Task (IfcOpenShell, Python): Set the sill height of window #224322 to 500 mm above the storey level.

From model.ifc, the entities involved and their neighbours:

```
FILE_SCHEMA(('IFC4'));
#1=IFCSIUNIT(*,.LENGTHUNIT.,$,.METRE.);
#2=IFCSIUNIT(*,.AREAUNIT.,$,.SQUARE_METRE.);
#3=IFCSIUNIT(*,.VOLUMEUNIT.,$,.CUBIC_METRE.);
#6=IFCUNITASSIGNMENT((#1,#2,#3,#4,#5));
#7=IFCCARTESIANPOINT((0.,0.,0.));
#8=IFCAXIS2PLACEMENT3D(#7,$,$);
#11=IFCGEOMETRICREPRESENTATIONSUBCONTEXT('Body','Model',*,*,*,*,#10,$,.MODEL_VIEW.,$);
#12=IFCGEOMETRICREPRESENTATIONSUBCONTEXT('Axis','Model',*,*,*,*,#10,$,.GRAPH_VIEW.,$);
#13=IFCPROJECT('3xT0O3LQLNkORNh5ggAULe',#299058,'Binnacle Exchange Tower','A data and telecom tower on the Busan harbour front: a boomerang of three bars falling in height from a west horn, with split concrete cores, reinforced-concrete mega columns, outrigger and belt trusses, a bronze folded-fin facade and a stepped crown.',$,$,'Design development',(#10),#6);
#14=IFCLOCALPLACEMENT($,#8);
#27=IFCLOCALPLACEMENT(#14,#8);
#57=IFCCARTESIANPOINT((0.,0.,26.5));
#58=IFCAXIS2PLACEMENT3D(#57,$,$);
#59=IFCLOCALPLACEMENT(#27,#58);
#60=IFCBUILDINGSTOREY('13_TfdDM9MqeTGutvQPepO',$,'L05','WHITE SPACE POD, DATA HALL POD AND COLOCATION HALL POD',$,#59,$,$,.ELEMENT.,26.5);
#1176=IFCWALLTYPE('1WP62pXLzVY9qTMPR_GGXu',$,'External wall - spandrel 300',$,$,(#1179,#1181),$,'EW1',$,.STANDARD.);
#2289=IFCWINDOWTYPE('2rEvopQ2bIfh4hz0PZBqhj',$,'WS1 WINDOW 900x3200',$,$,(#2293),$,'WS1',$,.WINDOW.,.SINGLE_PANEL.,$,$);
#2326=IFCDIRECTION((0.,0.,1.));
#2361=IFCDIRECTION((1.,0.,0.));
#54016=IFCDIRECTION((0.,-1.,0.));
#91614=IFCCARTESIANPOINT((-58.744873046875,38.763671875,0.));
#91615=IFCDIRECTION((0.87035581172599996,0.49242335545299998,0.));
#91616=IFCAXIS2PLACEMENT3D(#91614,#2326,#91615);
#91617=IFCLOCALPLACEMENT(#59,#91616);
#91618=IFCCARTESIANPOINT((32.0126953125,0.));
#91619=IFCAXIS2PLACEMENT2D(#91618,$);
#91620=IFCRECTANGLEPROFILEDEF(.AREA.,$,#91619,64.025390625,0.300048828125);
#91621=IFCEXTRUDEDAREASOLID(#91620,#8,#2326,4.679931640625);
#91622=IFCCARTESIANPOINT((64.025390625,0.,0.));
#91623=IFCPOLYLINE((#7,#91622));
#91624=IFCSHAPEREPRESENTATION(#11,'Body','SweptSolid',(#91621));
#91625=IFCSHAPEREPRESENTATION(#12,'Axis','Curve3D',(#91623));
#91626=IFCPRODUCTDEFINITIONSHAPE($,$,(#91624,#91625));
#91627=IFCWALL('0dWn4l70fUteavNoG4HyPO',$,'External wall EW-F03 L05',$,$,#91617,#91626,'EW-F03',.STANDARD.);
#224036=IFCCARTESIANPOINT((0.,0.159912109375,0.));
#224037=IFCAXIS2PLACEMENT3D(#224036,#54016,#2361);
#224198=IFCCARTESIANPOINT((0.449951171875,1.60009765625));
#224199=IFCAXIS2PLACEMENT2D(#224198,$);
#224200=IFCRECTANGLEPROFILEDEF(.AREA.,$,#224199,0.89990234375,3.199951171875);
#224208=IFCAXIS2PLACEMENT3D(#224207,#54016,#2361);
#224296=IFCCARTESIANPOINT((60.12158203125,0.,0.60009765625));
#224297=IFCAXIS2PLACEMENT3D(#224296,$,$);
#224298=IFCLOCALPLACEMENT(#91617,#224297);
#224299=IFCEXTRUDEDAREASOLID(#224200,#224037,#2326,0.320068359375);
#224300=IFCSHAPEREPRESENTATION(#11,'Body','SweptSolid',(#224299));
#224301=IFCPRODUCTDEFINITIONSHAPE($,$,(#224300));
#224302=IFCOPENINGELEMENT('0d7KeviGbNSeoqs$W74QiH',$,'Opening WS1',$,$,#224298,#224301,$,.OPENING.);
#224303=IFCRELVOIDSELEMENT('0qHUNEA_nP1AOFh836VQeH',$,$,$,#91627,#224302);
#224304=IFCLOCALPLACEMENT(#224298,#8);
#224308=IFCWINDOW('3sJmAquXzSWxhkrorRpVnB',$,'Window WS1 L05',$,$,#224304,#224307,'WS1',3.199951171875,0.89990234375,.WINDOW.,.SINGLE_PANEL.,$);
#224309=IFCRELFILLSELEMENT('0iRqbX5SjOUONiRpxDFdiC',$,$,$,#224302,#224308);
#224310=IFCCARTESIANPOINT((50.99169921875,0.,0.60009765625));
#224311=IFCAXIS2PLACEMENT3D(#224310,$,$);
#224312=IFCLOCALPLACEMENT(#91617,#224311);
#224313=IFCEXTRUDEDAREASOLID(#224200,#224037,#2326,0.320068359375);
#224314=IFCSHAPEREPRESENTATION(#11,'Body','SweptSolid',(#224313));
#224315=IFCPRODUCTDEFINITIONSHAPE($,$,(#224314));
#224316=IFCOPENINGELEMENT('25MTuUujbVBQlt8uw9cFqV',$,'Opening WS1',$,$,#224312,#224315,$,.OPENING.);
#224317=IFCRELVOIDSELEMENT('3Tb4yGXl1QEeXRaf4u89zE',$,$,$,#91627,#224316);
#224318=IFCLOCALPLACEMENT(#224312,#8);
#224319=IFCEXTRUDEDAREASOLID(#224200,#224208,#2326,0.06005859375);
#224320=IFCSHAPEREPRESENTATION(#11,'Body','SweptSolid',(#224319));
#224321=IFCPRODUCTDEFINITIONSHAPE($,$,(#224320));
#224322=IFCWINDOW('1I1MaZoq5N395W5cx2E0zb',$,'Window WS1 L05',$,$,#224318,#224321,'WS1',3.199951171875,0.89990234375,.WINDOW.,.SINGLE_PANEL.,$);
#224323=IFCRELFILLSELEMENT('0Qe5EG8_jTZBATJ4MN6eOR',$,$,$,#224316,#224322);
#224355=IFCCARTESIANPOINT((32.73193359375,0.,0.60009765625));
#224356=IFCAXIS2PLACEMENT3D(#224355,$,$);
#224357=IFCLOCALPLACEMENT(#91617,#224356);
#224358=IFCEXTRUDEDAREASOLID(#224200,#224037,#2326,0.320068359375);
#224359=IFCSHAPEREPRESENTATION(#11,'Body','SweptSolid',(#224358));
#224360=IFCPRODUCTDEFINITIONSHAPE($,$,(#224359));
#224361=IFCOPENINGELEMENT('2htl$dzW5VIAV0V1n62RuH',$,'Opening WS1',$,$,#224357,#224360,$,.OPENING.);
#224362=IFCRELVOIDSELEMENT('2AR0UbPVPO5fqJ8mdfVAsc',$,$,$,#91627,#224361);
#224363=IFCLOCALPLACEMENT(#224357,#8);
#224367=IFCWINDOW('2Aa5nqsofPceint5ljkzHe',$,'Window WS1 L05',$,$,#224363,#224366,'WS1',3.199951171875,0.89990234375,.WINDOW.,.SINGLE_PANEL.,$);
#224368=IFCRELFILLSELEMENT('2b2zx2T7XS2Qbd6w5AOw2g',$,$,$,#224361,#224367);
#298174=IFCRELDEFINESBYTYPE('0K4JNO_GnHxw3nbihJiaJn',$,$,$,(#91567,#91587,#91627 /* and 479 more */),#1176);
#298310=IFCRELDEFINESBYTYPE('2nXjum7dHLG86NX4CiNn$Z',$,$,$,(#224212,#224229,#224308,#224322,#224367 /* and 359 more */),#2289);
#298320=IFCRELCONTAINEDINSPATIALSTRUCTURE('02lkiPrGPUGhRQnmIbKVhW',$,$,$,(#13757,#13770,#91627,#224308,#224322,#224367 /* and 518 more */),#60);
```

```python
import numpy as np
import ifcopenshell
import ifcopenshell.api.geometry
import ifcopenshell.geom
import ifcopenshell.util.element
import ifcopenshell.util.placement
import ifcopenshell.util.shape
import ifcopenshell.util.unit

model = ifcopenshell.open("model.ifc")
unit_scale = ifcopenshell.util.unit.calculate_unit_scale(model)

window = model.by_guid("1I1MaZoq5N395W5cx2E0zb")
opening = window.FillsVoids[0].RelatingOpeningElement
storey = ifcopenshell.util.element.get_container(window, ifc_class="IfcBuildingStorey")
level = ifcopenshell.util.placement.get_local_placement(storey.ObjectPlacement)[2, 3]

# The opening's origin need not be at the sill, so measure its lowest point.
shape = ifcopenshell.geom.create_shape(ifcopenshell.geom.settings(), opening)
bottom = ifcopenshell.util.shape.get_shape_bottom_elevation(shape, shape.geometry) / unit_scale
dz = level + 0.5 - bottom

shift = np.array([0.0, 0.0, dz])
# The window is placed relative to its opening, so it follows when the opening moves.
matrix = ifcopenshell.util.placement.get_local_placement(opening.ObjectPlacement)
matrix[:3, 3] += shift
ifcopenshell.api.geometry.edit_object_placement(
    model, product=opening, matrix=matrix, is_si=False, should_transform_children=True
)

print(f"moved by {dz * unit_scale:+.3f} m")

model.write("model_v2.ifc")
```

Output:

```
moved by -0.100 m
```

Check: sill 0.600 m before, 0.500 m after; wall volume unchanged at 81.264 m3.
